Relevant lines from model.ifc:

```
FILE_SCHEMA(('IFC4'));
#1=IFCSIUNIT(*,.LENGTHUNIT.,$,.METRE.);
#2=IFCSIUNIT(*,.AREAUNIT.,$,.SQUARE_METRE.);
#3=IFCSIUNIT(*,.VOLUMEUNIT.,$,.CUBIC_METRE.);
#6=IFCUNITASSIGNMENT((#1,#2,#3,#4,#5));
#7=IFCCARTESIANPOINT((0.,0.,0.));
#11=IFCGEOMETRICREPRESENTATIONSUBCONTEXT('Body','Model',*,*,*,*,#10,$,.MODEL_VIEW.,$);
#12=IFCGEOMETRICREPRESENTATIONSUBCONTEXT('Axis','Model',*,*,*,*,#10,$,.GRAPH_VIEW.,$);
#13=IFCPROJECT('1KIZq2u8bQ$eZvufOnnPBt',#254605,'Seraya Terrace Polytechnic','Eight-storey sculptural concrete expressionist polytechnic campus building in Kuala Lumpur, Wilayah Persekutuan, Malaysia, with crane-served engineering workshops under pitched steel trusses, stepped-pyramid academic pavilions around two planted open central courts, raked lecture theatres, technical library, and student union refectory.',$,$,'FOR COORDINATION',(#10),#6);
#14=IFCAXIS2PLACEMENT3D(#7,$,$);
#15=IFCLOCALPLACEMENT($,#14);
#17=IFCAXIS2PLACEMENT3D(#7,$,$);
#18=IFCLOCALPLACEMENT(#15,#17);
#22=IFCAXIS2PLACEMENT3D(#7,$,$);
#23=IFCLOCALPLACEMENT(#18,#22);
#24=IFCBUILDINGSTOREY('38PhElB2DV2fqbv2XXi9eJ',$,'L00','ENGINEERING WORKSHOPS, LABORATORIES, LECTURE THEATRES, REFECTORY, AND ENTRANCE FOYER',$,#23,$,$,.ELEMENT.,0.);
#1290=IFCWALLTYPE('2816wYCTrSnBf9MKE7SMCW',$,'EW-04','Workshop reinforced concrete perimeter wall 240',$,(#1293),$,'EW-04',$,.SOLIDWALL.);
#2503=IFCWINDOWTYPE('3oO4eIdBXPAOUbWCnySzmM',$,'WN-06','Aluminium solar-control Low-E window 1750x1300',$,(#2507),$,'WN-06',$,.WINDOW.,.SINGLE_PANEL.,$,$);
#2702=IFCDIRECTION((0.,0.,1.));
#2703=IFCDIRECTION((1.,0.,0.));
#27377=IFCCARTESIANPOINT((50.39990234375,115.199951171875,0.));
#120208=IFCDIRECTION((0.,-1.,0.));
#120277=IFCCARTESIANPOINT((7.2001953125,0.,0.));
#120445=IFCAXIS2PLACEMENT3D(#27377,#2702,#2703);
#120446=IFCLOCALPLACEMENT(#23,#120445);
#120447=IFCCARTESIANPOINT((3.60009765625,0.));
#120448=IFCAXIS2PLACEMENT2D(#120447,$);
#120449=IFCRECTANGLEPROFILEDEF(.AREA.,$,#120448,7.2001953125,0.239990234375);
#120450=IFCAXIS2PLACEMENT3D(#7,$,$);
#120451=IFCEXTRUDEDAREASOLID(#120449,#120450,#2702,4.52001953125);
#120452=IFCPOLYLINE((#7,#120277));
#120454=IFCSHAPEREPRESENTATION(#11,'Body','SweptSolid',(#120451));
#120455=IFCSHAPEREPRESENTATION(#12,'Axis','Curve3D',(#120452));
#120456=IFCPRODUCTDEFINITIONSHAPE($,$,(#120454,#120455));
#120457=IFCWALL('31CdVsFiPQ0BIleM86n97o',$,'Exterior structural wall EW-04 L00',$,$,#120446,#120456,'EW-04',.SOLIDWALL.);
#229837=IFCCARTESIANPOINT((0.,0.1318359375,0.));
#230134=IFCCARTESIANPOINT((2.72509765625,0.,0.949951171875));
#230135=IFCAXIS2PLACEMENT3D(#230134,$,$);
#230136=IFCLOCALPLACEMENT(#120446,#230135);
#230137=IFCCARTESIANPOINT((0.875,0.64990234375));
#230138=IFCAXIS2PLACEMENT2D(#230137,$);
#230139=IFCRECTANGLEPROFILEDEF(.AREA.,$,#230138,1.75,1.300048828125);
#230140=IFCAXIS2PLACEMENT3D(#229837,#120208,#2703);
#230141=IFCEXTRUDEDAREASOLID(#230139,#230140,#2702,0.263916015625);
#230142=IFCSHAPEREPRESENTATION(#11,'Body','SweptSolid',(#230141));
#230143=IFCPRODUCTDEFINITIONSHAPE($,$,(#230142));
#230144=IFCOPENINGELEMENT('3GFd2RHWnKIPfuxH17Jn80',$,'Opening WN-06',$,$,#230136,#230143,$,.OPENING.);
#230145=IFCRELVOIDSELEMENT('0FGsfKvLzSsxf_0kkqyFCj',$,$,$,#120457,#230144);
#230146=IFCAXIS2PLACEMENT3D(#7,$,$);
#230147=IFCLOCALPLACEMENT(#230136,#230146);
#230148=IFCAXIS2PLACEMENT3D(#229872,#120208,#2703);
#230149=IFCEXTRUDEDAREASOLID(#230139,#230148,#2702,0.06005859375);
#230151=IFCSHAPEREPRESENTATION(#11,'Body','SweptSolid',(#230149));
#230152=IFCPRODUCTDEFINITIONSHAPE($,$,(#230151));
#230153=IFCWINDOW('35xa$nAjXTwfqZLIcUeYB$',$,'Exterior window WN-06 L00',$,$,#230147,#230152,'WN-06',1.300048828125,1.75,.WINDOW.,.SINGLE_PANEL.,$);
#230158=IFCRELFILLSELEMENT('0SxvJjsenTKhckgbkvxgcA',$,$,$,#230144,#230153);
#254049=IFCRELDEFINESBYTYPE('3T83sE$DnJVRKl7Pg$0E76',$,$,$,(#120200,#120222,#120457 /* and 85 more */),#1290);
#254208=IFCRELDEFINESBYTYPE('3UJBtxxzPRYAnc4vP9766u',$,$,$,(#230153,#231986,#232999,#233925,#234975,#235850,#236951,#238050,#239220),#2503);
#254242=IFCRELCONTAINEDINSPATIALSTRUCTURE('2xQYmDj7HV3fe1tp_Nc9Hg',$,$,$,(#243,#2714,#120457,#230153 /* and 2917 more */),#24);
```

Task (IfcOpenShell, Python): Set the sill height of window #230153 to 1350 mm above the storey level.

```python
import numpy as np
import ifcopenshell
import ifcopenshell.api.geometry
import ifcopenshell.geom
import ifcopenshell.util.element
import ifcopenshell.util.placement
import ifcopenshell.util.shape
import ifcopenshell.util.unit

model = ifcopenshell.open("model.ifc")
unit_scale = ifcopenshell.util.unit.calculate_unit_scale(model)

window = model.by_guid("35xa$nAjXTwfqZLIcUeYB$")
opening = window.FillsVoids[0].RelatingOpeningElement
storey = ifcopenshell.util.element.get_container(window, ifc_class="IfcBuildingStorey")
level = ifcopenshell.util.placement.get_local_placement(storey.ObjectPlacement)[2, 3]

# The opening's origin need not be at the sill, so measure its lowest point.
shape = ifcopenshell.geom.create_shape(ifcopenshell.geom.settings(), opening)
bottom = ifcopenshell.util.shape.get_shape_bottom_elevation(shape, shape.geometry) / unit_scale
dz = level + 1.35 / unit_scale - bottom

shift = np.array([0.0, 0.0, dz])
# The window is placed relative to its opening, so it follows when the opening moves.
matrix = ifcopenshell.util.placement.get_local_placement(opening.ObjectPlacement)
matrix[:3, 3] += shift
ifcopenshell.api.geometry.edit_object_placement(
    model, product=opening, matrix=matrix, is_si=False, should_transform_children=True
)

print(f"moved by {dz * unit_scale:+.3f} m")

model.write("model-out.ifc")
```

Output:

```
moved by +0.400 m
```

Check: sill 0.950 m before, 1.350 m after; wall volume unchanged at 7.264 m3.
